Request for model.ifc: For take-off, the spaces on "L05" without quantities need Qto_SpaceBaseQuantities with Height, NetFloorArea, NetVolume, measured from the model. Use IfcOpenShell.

First a look at what the model holds.

```python
import ifcopenshell
import ifcopenshell.util.element
import ifcopenshell.util.unit

model = ifcopenshell.open("model.ifc")
print(model.schema)
for unit_type in ("LENGTHUNIT", "AREAUNIT", "VOLUMEUNIT"):
    print(unit_type, ifcopenshell.util.unit.calculate_unit_scale(model, unit_type))
storey = next(s for s in model.by_type("IfcBuildingStorey") if s.Name == "L05")
spaces = [e for e in ifcopenshell.util.element.get_decomposition(storey) if e.is_a("IfcSpace")]
for e in sorted(spaces, key=lambda e: e.id()):
    print(e.id(), e.is_a(), e.Name, list(ifcopenshell.util.element.get_psets(e, qtos_only=True)), sep=" | ")
```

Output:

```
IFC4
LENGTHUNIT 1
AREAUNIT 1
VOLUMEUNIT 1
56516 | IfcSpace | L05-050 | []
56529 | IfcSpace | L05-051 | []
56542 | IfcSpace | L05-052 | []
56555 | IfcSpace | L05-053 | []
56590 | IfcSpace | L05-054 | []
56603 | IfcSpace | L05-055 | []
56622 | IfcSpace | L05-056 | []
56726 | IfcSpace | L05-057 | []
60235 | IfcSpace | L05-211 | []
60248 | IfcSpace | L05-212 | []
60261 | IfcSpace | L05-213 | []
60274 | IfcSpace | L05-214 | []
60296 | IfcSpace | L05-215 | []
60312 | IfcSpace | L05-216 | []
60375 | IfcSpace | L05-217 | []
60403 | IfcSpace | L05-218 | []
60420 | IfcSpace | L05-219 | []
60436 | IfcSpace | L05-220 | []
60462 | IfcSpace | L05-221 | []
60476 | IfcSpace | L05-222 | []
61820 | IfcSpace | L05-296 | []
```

```python
import ifcopenshell
import ifcopenshell.api.pset
import ifcopenshell.geom
import ifcopenshell.util.element
import ifcopenshell.util.shape
import ifcopenshell.util.unit

model = ifcopenshell.open("model.ifc")
unit_scale = ifcopenshell.util.unit.calculate_unit_scale(model)
area_scale = ifcopenshell.util.unit.calculate_unit_scale(model, "AREAUNIT")
volume_scale = ifcopenshell.util.unit.calculate_unit_scale(model, "VOLUMEUNIT")
settings = ifcopenshell.geom.settings()

storey = next(s for s in model.by_type("IfcBuildingStorey") if s.Name == "L05")
spaces = [e for e in ifcopenshell.util.element.get_decomposition(storey) if e.is_a("IfcSpace")]

for e in sorted(spaces, key=lambda e: e.id()):
    if ifcopenshell.util.element.get_psets(e, qtos_only=True, should_inherit=False):
        continue
    # Geometry comes back in metres, in the element's own axes.
    shape = ifcopenshell.geom.create_shape(settings, e)
    values = {
        "Height": ifcopenshell.util.shape.get_z(shape.geometry) / unit_scale,
        "NetFloorArea": ifcopenshell.util.shape.get_footprint_area(shape.geometry) / area_scale,
        "NetVolume": ifcopenshell.util.shape.get_volume(shape.geometry) / volume_scale,
    }
    qto = ifcopenshell.api.pset.add_qto(model, product=e, name="Qto_SpaceBaseQuantities")
    ifcopenshell.api.pset.edit_qto(model, qto=qto, properties=values)
    print(e.id(), {k: round(v, 3) for k, v in values.items()})

model.write("model_v2.ifc")
```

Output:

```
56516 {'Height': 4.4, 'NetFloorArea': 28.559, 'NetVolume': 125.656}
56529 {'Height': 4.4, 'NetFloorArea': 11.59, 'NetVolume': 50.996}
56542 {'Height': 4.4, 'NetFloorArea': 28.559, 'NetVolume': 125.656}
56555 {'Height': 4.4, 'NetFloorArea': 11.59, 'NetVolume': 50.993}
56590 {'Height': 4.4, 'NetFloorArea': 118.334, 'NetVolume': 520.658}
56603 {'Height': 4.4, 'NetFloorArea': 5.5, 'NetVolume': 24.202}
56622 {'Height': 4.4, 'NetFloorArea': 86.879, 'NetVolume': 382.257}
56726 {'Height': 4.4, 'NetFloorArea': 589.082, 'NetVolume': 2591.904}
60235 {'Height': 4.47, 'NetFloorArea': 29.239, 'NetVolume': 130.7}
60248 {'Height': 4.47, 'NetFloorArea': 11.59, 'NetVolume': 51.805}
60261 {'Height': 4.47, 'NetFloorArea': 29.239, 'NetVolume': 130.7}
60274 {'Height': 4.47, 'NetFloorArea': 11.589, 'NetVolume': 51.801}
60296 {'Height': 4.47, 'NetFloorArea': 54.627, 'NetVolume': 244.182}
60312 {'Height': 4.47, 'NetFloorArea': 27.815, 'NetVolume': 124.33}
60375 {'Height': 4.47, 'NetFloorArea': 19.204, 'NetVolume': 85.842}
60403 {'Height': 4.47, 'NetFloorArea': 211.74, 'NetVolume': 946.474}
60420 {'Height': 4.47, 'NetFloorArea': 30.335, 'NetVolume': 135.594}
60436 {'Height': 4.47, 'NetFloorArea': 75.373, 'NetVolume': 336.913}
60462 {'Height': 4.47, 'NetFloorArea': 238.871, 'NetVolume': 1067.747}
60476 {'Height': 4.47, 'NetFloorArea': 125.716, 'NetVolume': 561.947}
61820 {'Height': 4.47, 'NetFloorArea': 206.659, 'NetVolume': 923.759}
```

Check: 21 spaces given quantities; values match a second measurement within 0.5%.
